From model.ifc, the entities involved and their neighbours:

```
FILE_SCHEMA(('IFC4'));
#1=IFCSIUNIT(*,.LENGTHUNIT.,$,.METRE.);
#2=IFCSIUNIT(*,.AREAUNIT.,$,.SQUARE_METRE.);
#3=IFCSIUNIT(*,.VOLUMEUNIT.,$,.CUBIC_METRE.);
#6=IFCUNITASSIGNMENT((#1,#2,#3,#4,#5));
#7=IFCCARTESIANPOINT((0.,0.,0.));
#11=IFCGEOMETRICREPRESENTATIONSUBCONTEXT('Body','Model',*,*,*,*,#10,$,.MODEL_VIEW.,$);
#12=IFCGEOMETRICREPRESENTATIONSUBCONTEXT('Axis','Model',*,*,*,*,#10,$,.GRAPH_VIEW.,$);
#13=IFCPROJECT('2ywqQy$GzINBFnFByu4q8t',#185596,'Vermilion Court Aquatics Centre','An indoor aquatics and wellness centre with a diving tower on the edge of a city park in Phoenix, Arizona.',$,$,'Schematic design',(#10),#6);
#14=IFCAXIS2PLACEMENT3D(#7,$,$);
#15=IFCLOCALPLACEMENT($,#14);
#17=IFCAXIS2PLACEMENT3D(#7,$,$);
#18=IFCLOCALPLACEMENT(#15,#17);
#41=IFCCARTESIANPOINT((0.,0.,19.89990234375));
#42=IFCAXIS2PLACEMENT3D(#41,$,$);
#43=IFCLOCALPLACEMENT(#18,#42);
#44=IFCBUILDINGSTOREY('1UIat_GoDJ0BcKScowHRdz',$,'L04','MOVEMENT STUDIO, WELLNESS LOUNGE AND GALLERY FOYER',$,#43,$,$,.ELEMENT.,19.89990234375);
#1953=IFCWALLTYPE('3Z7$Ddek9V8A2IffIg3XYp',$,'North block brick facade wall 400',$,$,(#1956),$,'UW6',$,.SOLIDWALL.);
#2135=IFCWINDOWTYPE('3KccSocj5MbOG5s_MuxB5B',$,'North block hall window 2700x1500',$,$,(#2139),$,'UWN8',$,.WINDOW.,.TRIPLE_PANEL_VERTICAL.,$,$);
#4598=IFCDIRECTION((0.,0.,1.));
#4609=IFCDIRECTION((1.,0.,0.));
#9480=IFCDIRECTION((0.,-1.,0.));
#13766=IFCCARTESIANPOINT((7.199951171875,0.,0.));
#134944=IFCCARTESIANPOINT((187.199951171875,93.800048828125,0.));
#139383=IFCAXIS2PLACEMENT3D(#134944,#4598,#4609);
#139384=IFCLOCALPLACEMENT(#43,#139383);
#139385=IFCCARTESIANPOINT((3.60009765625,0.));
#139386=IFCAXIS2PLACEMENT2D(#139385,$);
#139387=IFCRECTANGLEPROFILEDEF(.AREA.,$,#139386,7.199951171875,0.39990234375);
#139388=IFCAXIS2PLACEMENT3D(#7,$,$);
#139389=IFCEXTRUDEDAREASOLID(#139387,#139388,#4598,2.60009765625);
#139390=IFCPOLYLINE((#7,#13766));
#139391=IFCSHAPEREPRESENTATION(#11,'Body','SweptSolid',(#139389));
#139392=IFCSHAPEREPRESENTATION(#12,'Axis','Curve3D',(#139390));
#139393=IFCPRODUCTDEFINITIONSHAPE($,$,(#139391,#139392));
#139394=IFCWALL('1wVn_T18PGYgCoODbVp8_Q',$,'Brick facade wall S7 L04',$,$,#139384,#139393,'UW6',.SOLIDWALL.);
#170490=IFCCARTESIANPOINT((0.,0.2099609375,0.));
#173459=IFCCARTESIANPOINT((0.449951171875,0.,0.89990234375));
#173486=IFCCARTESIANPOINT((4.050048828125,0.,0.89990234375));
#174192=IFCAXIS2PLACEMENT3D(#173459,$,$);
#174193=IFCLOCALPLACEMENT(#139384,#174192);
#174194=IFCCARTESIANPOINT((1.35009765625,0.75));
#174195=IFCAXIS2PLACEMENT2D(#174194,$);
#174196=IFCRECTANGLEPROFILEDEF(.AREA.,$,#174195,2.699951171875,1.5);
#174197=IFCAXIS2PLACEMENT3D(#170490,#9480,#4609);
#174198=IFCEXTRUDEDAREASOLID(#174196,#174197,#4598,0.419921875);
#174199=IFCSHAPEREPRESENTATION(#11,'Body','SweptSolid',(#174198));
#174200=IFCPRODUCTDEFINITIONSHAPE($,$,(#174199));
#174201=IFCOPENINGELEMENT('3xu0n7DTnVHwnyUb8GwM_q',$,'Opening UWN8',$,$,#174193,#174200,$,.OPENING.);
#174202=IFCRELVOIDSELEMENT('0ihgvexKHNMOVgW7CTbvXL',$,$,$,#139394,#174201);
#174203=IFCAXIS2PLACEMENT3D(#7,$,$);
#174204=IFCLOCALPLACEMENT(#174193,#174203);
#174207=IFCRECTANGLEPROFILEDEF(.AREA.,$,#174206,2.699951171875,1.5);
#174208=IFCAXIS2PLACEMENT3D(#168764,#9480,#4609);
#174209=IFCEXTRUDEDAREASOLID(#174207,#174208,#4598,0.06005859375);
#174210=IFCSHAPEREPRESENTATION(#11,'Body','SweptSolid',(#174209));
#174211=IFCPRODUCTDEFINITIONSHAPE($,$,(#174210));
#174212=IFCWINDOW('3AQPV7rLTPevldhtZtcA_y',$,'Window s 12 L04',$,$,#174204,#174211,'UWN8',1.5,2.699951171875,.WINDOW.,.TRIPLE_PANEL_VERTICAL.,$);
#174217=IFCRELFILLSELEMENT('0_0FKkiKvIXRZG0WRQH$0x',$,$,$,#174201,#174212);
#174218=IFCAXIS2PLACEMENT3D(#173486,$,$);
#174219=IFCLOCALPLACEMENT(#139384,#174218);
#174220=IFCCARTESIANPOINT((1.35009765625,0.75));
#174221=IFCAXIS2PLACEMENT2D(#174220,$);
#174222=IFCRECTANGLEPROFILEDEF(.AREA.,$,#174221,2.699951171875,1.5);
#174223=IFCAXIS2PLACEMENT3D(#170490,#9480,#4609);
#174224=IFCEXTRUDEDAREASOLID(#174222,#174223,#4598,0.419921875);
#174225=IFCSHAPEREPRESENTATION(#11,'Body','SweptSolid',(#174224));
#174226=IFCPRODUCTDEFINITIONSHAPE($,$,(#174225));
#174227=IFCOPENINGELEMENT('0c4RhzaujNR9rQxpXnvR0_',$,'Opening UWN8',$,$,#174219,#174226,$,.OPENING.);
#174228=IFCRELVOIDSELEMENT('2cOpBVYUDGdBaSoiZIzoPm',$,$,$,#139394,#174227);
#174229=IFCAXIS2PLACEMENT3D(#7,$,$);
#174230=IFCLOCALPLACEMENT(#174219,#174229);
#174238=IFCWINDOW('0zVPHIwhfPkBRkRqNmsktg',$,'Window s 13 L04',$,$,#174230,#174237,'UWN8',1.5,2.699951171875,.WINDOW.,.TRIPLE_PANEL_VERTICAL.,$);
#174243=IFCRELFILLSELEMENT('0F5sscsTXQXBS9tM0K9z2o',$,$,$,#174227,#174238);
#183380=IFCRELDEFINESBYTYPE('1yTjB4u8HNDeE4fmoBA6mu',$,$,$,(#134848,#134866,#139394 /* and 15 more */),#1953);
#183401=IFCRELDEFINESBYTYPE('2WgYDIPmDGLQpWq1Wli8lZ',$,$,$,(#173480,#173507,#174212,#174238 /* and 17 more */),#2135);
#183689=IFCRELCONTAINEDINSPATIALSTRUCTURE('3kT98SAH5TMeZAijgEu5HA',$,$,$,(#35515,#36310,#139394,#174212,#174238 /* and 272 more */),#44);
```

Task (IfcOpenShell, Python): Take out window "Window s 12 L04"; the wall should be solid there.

```python
import ifcopenshell
import ifcopenshell.api.feature
import ifcopenshell.api.root
import ifcopenshell.geom
import ifcopenshell.util.shape

model = ifcopenshell.open("model.ifc")
settings = ifcopenshell.geom.settings()


def volume(element):
    """Net volume in cubic metres, openings subtracted."""
    shape = ifcopenshell.geom.create_shape(settings, element)
    return ifcopenshell.util.shape.get_volume(shape.geometry)


window = model.by_guid("3AQPV7rLTPevldhtZtcA_y")
opening = window.FillsVoids[0].RelatingOpeningElement
wall = opening.VoidsElements[0].RelatingBuildingElement
before = volume(wall)

ifcopenshell.api.root.remove_product(model, product=window)
ifcopenshell.api.feature.remove_feature(model, feature=opening)

after = volume(wall)

print(f"wall volume {before:.3f} -> {after:.3f} m3")

model.write("model_rev.ifc")
```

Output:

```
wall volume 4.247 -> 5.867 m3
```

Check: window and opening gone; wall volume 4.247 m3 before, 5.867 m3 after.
